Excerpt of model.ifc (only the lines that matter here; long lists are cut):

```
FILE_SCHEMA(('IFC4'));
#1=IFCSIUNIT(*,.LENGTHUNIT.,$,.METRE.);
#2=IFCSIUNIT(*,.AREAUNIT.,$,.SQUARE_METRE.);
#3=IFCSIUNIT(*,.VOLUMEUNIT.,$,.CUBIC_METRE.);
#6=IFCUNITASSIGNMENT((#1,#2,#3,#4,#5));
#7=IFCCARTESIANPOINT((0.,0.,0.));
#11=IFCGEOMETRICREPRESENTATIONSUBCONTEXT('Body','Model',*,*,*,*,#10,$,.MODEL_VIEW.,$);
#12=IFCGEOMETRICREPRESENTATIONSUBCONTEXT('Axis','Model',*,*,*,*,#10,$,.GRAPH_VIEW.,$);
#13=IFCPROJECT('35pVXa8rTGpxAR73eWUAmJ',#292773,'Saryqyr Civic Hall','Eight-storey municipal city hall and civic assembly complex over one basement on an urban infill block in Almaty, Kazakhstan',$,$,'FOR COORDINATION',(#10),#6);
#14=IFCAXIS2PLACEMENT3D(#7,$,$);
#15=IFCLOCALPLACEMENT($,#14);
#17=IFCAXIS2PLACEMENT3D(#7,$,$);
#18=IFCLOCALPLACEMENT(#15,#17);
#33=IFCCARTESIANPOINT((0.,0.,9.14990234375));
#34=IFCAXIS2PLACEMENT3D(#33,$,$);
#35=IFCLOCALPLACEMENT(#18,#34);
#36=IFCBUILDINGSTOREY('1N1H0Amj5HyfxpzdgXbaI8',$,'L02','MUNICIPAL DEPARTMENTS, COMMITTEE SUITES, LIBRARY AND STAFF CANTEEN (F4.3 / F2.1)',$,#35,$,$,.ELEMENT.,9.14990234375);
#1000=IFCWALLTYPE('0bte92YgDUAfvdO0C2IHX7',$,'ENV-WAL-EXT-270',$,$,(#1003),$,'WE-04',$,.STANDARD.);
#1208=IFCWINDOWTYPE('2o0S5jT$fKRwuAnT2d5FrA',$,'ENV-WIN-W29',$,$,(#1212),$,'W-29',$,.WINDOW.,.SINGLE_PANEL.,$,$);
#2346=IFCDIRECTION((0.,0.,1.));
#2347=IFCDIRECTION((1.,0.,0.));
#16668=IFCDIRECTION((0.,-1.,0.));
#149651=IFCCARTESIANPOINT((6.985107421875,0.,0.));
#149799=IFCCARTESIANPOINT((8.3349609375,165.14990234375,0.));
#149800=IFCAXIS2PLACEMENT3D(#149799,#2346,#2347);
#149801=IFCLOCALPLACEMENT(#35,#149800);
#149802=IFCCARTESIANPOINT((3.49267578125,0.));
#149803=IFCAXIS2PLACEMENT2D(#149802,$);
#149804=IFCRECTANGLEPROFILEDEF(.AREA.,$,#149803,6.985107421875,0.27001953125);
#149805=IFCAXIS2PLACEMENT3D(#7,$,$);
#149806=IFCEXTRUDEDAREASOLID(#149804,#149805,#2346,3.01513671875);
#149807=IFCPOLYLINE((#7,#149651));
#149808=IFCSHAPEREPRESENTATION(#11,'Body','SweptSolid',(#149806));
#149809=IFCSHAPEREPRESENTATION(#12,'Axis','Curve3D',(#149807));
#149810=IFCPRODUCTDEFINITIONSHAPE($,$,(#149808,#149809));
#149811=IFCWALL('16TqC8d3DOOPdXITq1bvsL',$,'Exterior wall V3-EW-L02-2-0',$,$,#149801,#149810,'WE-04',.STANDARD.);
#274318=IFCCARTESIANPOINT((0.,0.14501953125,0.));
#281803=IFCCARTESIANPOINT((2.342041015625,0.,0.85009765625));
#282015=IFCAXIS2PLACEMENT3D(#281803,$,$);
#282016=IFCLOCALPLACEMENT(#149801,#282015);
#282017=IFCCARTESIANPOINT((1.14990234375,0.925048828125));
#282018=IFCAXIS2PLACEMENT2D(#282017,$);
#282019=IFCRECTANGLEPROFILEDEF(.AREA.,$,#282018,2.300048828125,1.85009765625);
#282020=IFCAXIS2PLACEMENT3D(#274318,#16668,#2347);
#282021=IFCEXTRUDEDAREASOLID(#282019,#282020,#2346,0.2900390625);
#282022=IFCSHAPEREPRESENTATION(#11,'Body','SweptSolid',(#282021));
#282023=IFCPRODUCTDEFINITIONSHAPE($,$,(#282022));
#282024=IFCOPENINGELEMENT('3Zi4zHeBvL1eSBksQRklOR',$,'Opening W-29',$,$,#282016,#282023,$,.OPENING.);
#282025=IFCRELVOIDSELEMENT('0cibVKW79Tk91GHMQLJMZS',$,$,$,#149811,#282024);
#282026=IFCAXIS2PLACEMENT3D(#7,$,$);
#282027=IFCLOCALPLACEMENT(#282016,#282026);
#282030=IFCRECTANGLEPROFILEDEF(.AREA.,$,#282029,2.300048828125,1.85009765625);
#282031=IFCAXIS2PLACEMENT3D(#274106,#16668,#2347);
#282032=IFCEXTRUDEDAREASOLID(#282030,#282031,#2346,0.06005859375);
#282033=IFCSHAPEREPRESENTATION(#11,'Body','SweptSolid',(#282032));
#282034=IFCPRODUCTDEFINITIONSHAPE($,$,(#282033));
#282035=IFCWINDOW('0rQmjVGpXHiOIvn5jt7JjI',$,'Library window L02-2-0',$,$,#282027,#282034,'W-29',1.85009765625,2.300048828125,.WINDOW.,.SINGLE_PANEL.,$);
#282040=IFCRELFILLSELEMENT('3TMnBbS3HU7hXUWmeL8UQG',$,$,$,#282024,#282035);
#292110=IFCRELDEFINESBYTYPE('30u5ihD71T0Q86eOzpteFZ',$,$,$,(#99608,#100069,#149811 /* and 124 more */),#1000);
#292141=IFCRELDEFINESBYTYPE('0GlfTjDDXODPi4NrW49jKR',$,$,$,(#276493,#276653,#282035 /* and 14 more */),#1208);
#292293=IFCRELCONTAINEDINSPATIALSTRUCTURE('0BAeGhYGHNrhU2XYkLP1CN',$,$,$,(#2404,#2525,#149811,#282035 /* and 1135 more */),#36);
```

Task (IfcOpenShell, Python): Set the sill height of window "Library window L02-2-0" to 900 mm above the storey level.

```python
import numpy as np
import ifcopenshell
import ifcopenshell.api.geometry
import ifcopenshell.geom
import ifcopenshell.util.element
import ifcopenshell.util.placement
import ifcopenshell.util.shape
import ifcopenshell.util.unit

model = ifcopenshell.open("model.ifc")
unit_scale = ifcopenshell.util.unit.calculate_unit_scale(model)

window = model.by_id(282035)
opening = window.FillsVoids[0].RelatingOpeningElement
storey = ifcopenshell.util.element.get_container(window, ifc_class="IfcBuildingStorey")
level = ifcopenshell.util.placement.get_local_placement(storey.ObjectPlacement)[2, 3]

# The opening's origin need not be at the sill, so measure its lowest point.
shape = ifcopenshell.geom.create_shape(ifcopenshell.geom.settings(), opening)
bottom = ifcopenshell.util.shape.get_shape_bottom_elevation(shape, shape.geometry) / unit_scale
dz = level + 0.9 - bottom

shift = np.array([0.0, 0.0, dz])
# The window is placed relative to its opening, so it follows when the opening moves.
matrix = ifcopenshell.util.placement.get_local_placement(opening.ObjectPlacement)
matrix[:3, 3] += shift
ifcopenshell.api.geometry.edit_object_placement(
    model, product=opening, matrix=matrix, is_si=False, should_transform_children=True
)

print(f"moved by {dz * unit_scale:+.3f} m")

model.write("model_updated.ifc")
```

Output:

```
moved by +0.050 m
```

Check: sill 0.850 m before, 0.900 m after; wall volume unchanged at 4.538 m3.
